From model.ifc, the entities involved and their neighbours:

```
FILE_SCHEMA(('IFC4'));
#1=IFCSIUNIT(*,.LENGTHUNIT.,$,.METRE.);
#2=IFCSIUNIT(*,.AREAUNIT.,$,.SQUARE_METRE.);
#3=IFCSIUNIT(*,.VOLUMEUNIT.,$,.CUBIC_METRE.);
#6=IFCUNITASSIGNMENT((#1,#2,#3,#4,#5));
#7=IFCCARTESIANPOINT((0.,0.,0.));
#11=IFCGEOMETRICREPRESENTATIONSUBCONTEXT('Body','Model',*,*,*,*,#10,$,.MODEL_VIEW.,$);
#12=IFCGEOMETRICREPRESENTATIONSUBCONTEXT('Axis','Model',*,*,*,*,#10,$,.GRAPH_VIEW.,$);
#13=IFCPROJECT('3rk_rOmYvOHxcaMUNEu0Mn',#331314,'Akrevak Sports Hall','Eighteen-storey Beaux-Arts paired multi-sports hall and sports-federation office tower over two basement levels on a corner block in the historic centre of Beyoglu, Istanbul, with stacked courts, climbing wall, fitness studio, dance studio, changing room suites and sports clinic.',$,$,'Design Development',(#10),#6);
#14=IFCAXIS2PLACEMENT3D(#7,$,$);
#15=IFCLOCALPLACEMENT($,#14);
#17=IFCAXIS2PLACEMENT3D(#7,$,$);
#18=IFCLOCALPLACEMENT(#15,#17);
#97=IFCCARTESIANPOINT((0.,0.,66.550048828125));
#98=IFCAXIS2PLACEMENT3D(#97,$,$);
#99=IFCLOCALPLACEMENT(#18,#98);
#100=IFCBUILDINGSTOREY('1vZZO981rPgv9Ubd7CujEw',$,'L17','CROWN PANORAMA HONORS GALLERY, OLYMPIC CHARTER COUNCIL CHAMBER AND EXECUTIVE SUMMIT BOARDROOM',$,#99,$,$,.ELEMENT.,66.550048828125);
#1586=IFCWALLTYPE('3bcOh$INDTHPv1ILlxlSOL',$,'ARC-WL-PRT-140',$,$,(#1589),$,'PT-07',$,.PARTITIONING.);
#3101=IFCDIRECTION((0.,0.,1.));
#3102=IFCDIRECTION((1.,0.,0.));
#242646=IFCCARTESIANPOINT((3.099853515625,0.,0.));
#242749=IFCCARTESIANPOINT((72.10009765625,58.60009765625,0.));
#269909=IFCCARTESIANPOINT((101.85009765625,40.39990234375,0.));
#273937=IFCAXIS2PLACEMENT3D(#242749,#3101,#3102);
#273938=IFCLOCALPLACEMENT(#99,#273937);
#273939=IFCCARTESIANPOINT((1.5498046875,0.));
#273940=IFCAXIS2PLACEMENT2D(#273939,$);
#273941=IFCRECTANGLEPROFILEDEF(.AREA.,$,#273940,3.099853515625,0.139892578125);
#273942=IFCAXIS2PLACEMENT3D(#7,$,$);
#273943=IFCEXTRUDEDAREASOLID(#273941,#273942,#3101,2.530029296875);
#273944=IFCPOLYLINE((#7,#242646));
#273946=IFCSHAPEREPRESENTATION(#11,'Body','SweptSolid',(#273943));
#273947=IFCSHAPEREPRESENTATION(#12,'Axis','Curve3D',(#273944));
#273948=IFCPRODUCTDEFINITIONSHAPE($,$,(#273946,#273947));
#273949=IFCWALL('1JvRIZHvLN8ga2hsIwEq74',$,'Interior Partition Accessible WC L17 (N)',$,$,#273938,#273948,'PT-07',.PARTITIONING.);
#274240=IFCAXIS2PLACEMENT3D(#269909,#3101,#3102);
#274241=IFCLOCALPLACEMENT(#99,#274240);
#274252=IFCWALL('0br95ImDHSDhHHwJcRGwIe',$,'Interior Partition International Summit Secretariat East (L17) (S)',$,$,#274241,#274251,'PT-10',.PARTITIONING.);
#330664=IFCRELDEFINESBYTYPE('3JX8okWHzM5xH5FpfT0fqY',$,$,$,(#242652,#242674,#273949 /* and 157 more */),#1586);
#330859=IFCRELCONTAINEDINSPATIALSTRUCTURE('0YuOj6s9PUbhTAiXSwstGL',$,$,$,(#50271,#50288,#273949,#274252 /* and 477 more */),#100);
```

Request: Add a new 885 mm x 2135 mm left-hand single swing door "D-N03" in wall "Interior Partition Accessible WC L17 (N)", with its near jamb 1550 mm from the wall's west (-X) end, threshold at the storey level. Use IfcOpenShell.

```python
import numpy as np
import ifcopenshell
import ifcopenshell.api.feature
import ifcopenshell.api.geometry
import ifcopenshell.api.root
import ifcopenshell.api.spatial
import ifcopenshell.geom
import ifcopenshell.util.element
import ifcopenshell.util.placement
import ifcopenshell.util.representation
import ifcopenshell.util.shape
import ifcopenshell.util.unit

model = ifcopenshell.open("model.ifc")
unit_scale = ifcopenshell.util.unit.calculate_unit_scale(model)
settings = ifcopenshell.geom.settings()


def volume(element):
    """Net volume in cubic metres, openings subtracted."""
    shape = ifcopenshell.geom.create_shape(settings, element)
    return ifcopenshell.util.shape.get_volume(shape.geometry)


wall = model.by_id(273949)
storey = ifcopenshell.util.element.get_container(wall, ifc_class="IfcBuildingStorey")
context = ifcopenshell.util.representation.get_context(model, "Model", "Body", "MODEL_VIEW")
before = volume(wall)

width, height, from_end, sill = 0.885, 2.135, 1.55, 0.0  # metres

# The wall runs along its own X axis, and the end named is its -X end.
wall_shape = ifcopenshell.geom.create_shape(settings, wall)
x, y, z = ifcopenshell.util.shape.get_vertices(wall_shape.geometry).T
start = x.min() + from_end
face, thickness = float(y.min()), float(y.max() - y.min())
wall_matrix = ifcopenshell.util.placement.get_local_placement(wall.ObjectPlacement)
level = ifcopenshell.util.placement.get_local_placement(storey.ObjectPlacement)[2, 3]


def in_wall(x, y):
    """Placement at x, y metres in the wall's axes, at sill height."""
    matrix = wall_matrix.copy()
    matrix[:, 3] = wall_matrix @ np.array([x / unit_scale, y / unit_scale, 0.0, 1.0])
    matrix[2, 3] = level + sill / unit_scale
    return matrix


# Opening: a box that overshoots both wall faces by 50 mm.
opening = ifcopenshell.api.root.create_entity(model, ifc_class="IfcOpeningElement", predefined_type="OPENING")
box = ifcopenshell.api.geometry.add_wall_representation(
    model, context=context, length=width, height=height, thickness=thickness + 0.1
)
ifcopenshell.api.geometry.assign_representation(model, product=opening, representation=box)
ifcopenshell.api.geometry.edit_object_placement(model, product=opening, matrix=in_wall(start, face - 0.05), is_si=False)
ifcopenshell.api.feature.add_feature(model, feature=opening, element=wall)

door = ifcopenshell.api.root.create_entity(model, ifc_class="IfcDoor", name="D-N03", predefined_type="DOOR")
door.OverallWidth, door.OverallHeight = width / unit_scale, height / unit_scale
door.OperationType = "SINGLE_SWING_LEFT"
body = ifcopenshell.api.geometry.add_door_representation(
    model,
    context=context,
    overall_width=door.OverallWidth,
    overall_height=door.OverallHeight,
    operation_type="SINGLE_SWING_LEFT",
    lining_properties={"LiningDepth": thickness / unit_scale, "ThresholdDepth": thickness / unit_scale},
)
ifcopenshell.api.geometry.assign_representation(model, product=door, representation=body)
ifcopenshell.api.spatial.assign_container(model, products=[door], relating_structure=storey)
ifcopenshell.api.feature.add_filling(model, opening=opening, element=door)

# The lining spans the wall, so the door starts at the wall face.
ifcopenshell.api.geometry.edit_object_placement(model, product=door, matrix=in_wall(start, face), is_si=False)

after = volume(wall)

print(f"wall volume {before:.3f} -> {after:.3f} m3")

model.write("model_v2.ifc")
```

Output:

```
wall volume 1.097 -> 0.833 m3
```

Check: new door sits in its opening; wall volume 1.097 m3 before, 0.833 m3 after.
